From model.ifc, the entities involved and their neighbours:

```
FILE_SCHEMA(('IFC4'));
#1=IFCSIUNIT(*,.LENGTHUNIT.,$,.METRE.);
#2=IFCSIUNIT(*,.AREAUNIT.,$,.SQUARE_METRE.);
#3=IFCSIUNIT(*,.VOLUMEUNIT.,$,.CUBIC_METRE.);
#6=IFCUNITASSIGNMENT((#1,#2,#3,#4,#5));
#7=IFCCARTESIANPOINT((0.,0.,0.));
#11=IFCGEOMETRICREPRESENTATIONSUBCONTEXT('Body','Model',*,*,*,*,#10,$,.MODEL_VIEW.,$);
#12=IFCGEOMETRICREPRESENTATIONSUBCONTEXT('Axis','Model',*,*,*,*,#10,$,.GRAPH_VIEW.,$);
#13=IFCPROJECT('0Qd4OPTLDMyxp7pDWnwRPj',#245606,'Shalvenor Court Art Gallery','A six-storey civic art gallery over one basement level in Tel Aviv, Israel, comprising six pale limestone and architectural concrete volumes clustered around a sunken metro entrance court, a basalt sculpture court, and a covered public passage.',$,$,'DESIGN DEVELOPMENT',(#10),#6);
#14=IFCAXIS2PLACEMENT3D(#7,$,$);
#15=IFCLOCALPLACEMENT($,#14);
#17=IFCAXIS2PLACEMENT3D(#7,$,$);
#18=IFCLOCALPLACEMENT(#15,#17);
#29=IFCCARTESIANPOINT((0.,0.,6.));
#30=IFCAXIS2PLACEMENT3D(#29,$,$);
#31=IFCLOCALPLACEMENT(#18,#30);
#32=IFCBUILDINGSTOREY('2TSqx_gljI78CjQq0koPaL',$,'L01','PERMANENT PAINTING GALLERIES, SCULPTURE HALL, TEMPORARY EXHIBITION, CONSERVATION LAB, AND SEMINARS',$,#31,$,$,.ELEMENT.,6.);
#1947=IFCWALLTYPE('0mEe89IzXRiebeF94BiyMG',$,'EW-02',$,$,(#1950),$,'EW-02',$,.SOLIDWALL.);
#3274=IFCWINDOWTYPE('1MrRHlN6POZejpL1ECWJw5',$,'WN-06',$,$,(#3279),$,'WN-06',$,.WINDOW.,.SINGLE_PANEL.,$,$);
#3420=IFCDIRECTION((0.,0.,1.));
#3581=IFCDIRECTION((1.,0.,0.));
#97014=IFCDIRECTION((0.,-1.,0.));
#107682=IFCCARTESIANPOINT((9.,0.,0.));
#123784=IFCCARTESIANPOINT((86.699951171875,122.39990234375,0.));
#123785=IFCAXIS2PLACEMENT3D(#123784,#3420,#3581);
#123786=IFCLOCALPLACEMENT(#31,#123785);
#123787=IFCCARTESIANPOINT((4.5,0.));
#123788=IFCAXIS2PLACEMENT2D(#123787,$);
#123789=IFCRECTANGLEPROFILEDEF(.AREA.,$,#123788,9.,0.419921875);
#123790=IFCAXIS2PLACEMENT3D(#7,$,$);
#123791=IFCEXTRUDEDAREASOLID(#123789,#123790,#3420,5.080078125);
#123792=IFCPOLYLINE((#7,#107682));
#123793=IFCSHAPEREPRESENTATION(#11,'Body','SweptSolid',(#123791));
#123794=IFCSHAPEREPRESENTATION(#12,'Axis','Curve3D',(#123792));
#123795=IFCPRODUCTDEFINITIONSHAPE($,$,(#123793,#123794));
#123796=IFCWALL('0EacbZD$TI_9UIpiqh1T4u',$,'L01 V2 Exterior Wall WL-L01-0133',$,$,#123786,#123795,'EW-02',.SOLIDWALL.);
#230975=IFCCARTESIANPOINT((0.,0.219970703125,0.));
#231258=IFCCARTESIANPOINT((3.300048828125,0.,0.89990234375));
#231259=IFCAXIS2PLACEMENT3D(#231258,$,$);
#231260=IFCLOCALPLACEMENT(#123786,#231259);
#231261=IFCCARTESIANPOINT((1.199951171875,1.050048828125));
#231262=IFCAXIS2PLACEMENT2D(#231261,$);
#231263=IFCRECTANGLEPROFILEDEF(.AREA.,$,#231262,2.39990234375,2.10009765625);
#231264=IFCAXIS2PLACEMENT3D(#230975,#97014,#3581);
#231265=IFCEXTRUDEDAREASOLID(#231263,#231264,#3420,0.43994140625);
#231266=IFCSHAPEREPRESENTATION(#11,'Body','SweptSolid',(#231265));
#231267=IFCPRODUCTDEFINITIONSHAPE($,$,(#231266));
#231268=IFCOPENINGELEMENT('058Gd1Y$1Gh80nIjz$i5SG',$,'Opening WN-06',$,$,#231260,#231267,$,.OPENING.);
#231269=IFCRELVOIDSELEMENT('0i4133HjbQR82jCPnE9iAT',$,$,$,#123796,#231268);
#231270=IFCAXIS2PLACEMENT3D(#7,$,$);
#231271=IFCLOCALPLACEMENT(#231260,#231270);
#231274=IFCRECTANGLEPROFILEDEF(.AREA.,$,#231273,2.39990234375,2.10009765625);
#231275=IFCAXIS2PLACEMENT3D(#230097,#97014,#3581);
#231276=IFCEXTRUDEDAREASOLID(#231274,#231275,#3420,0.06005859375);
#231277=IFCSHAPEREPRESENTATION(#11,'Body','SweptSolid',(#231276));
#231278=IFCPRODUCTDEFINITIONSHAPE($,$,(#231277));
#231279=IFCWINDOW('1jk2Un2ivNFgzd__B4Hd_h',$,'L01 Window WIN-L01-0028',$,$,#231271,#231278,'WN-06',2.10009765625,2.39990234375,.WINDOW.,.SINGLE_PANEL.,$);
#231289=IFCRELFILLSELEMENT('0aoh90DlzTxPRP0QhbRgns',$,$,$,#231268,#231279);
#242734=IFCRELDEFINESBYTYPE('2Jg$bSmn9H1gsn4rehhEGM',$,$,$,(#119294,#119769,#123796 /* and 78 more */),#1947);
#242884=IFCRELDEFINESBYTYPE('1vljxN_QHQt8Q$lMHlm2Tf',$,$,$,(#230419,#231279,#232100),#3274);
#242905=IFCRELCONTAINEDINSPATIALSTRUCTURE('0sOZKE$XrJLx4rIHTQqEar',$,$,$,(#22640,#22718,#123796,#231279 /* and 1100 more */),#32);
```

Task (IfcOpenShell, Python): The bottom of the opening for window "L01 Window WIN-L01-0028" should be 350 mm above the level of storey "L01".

```python
import numpy as np
import ifcopenshell
import ifcopenshell.api.geometry
import ifcopenshell.geom
import ifcopenshell.util.element
import ifcopenshell.util.placement
import ifcopenshell.util.shape
import ifcopenshell.util.unit

model = ifcopenshell.open("model.ifc")
unit_scale = ifcopenshell.util.unit.calculate_unit_scale(model)

window = model.by_guid("1jk2Un2ivNFgzd__B4Hd_h")
opening = window.FillsVoids[0].RelatingOpeningElement
storey = ifcopenshell.util.element.get_container(window, ifc_class="IfcBuildingStorey")
level = ifcopenshell.util.placement.get_local_placement(storey.ObjectPlacement)[2, 3]

# The opening's origin need not be at the sill, so measure its lowest point.
shape = ifcopenshell.geom.create_shape(ifcopenshell.geom.settings(), opening)
bottom = ifcopenshell.util.shape.get_shape_bottom_elevation(shape, shape.geometry) / unit_scale
dz = level + 0.35 / unit_scale - bottom

shift = np.array([0.0, 0.0, dz])
# The window is placed relative to its opening, so it follows when the opening moves.
matrix = ifcopenshell.util.placement.get_local_placement(opening.ObjectPlacement)
matrix[:3, 3] += shift
ifcopenshell.api.geometry.edit_object_placement(
    model, product=opening, matrix=matrix, is_si=False, should_transform_children=True
)

print(f"moved by {dz * unit_scale:+.3f} m")

model.write("model_v2.ifc")
```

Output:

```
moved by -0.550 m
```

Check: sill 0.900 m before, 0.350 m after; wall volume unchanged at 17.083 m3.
